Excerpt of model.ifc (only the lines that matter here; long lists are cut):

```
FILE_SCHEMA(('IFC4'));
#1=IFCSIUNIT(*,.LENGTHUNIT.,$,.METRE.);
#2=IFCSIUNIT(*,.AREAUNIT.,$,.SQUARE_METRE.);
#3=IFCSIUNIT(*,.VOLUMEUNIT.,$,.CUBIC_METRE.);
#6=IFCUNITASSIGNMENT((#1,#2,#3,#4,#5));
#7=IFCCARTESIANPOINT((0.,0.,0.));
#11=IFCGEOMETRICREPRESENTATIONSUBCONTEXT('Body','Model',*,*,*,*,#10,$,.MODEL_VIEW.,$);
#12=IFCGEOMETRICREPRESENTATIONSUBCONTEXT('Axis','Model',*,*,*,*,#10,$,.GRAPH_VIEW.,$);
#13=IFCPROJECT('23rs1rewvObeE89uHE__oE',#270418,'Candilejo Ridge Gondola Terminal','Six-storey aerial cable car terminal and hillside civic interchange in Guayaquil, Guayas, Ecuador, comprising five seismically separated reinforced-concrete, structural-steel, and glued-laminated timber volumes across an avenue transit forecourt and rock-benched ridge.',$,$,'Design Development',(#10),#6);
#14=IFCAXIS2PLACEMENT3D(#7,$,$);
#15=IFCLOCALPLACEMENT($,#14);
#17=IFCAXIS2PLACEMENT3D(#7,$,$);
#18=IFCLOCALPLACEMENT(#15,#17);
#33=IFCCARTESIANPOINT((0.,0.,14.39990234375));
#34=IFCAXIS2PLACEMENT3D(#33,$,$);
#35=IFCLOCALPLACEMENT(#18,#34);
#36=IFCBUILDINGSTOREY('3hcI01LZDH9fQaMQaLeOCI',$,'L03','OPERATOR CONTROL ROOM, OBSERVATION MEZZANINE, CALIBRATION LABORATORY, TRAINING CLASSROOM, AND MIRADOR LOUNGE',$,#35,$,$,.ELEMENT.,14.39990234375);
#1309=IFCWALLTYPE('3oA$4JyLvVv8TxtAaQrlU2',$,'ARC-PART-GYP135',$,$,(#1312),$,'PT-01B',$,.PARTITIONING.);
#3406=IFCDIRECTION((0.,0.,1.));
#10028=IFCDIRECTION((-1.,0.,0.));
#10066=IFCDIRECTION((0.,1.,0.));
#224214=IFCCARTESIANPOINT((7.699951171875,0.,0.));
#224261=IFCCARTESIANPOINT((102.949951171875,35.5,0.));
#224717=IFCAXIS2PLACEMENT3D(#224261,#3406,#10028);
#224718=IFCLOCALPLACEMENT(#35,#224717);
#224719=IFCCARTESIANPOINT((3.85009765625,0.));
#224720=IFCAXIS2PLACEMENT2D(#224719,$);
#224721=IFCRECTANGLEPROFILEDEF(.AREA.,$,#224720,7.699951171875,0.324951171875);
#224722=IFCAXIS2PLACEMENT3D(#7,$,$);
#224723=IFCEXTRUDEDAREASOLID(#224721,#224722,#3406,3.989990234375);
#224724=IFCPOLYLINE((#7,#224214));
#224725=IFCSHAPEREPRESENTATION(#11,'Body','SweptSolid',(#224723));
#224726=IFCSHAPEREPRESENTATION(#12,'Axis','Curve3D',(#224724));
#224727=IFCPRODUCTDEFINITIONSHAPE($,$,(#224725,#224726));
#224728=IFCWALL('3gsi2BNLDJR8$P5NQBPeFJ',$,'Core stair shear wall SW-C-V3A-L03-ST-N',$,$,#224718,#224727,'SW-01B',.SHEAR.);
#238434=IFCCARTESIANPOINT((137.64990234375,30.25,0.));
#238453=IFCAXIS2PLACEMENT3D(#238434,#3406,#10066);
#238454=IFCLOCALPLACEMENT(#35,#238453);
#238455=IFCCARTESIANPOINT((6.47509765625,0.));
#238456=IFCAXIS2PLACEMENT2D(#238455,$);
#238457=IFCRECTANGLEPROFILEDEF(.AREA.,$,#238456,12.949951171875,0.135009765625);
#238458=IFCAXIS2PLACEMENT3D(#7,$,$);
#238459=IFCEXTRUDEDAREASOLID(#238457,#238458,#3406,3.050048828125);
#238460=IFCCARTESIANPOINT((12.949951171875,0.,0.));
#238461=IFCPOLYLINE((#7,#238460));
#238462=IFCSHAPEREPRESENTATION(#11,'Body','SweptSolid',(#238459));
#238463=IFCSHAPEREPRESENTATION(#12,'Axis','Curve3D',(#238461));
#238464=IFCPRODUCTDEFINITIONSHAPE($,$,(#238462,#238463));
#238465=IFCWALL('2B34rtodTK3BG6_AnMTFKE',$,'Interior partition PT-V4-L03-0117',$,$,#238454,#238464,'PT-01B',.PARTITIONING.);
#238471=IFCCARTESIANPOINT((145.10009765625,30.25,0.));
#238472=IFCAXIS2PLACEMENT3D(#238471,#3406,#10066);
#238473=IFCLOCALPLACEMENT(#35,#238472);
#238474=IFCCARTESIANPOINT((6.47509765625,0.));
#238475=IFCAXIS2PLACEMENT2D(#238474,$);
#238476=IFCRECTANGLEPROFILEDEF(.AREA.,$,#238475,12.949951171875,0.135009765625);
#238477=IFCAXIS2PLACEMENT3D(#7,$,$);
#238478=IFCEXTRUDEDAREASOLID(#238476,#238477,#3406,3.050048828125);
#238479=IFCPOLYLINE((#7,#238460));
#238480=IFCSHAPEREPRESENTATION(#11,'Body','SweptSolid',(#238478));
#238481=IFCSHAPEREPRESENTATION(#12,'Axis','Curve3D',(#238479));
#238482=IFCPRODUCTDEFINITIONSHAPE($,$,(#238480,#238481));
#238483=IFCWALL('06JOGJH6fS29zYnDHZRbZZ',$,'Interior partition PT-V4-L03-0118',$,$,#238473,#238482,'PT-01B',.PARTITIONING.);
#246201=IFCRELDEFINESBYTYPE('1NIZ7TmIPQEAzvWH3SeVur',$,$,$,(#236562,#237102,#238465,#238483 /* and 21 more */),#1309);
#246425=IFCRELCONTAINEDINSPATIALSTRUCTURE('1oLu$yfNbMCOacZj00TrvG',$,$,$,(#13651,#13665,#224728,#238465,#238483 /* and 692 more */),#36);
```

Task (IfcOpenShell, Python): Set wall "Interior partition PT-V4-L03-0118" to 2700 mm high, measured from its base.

```python
import ifcopenshell
import ifcopenshell.geom
import ifcopenshell.util.representation
import ifcopenshell.util.shape
import ifcopenshell.util.unit

model = ifcopenshell.open("model.ifc")
unit_scale = ifcopenshell.util.unit.calculate_unit_scale(model)
settings = ifcopenshell.geom.settings()


def volume(element):
    """Net volume in cubic metres, openings subtracted."""
    shape = ifcopenshell.geom.create_shape(settings, element)
    return ifcopenshell.util.shape.get_volume(shape.geometry)


wall = model.by_id(238483)
before = volume(wall)

body = ifcopenshell.util.representation.get_representation(wall, "Model", "Body")
solid = body.Items[0]
old_height = solid.Depth
solid.Depth = 2.7 / unit_scale
after = volume(wall)

print(f"height {old_height:g} -> {solid.Depth:g}, volume {before:.3f} -> {after:.3f} m3")

model.write("model-out.ifc")
```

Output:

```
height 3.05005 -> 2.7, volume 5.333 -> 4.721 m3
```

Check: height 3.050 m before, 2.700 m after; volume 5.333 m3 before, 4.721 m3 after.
